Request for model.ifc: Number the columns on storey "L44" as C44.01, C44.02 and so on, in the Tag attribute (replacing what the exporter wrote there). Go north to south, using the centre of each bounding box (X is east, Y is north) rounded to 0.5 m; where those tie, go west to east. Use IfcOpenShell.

First a look at what the model holds.

```python
import ifcopenshell
import ifcopenshell.util.element
import ifcopenshell.util.placement

model = ifcopenshell.open("model.ifc")
print(model.schema)
storey = next(s for s in model.by_type("IfcBuildingStorey") if s.Name == "L44")
columns = [e for e in ifcopenshell.util.element.get_decomposition(storey) if e.is_a("IfcColumn")]
for e in sorted(columns, key=lambda e: e.id()):
    origin = ifcopenshell.util.placement.get_local_placement(e.ObjectPlacement)[:3, 3]
    print(e.id(), e.Tag, e.Name, origin.round(2) + 0.0, sep=" | ")
```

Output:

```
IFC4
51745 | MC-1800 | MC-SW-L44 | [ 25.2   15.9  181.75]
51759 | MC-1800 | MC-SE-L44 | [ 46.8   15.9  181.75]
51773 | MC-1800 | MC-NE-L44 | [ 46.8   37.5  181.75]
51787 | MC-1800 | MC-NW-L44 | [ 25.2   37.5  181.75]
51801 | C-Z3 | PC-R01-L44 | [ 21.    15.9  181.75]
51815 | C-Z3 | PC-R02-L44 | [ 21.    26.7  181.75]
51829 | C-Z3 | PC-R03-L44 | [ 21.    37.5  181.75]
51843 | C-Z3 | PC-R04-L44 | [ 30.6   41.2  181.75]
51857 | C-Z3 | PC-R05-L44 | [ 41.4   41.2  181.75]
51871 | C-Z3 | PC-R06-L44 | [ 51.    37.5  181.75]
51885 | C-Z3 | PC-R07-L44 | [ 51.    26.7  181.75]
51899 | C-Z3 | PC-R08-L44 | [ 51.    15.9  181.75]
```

```python
import ifcopenshell
import ifcopenshell.geom
import ifcopenshell.util.element
import ifcopenshell.util.shape

model = ifcopenshell.open("model.ifc")
settings = ifcopenshell.geom.settings()
settings.set("use-world-coords", True)


def centre(element):
    shape = ifcopenshell.geom.create_shape(settings, element)
    return ifcopenshell.util.shape.get_bbox_centroid(shape.geometry)


storey = next(s for s in model.by_type("IfcBuildingStorey") if s.Name == "L44")
columns = [e for e in ifcopenshell.util.element.get_decomposition(storey) if e.is_a("IfcColumn")]

# Insertion points can sit at a corner or the storey origin, so sort by the geometry (in metres).
centres = {e: centre(e) for e in columns}
columns.sort(key=lambda e: (-round(centres[e][1] / 0.5), centres[e][0]))

for i, e in enumerate(columns, start=1):
    number = f"C44.{i:02d}"
    e.Tag = number
    print(e.id(), number)

model.write("model_edited.ifc")
```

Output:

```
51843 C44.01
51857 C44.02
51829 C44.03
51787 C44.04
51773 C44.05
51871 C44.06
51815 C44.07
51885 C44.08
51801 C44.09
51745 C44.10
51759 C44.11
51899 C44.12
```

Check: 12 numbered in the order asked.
